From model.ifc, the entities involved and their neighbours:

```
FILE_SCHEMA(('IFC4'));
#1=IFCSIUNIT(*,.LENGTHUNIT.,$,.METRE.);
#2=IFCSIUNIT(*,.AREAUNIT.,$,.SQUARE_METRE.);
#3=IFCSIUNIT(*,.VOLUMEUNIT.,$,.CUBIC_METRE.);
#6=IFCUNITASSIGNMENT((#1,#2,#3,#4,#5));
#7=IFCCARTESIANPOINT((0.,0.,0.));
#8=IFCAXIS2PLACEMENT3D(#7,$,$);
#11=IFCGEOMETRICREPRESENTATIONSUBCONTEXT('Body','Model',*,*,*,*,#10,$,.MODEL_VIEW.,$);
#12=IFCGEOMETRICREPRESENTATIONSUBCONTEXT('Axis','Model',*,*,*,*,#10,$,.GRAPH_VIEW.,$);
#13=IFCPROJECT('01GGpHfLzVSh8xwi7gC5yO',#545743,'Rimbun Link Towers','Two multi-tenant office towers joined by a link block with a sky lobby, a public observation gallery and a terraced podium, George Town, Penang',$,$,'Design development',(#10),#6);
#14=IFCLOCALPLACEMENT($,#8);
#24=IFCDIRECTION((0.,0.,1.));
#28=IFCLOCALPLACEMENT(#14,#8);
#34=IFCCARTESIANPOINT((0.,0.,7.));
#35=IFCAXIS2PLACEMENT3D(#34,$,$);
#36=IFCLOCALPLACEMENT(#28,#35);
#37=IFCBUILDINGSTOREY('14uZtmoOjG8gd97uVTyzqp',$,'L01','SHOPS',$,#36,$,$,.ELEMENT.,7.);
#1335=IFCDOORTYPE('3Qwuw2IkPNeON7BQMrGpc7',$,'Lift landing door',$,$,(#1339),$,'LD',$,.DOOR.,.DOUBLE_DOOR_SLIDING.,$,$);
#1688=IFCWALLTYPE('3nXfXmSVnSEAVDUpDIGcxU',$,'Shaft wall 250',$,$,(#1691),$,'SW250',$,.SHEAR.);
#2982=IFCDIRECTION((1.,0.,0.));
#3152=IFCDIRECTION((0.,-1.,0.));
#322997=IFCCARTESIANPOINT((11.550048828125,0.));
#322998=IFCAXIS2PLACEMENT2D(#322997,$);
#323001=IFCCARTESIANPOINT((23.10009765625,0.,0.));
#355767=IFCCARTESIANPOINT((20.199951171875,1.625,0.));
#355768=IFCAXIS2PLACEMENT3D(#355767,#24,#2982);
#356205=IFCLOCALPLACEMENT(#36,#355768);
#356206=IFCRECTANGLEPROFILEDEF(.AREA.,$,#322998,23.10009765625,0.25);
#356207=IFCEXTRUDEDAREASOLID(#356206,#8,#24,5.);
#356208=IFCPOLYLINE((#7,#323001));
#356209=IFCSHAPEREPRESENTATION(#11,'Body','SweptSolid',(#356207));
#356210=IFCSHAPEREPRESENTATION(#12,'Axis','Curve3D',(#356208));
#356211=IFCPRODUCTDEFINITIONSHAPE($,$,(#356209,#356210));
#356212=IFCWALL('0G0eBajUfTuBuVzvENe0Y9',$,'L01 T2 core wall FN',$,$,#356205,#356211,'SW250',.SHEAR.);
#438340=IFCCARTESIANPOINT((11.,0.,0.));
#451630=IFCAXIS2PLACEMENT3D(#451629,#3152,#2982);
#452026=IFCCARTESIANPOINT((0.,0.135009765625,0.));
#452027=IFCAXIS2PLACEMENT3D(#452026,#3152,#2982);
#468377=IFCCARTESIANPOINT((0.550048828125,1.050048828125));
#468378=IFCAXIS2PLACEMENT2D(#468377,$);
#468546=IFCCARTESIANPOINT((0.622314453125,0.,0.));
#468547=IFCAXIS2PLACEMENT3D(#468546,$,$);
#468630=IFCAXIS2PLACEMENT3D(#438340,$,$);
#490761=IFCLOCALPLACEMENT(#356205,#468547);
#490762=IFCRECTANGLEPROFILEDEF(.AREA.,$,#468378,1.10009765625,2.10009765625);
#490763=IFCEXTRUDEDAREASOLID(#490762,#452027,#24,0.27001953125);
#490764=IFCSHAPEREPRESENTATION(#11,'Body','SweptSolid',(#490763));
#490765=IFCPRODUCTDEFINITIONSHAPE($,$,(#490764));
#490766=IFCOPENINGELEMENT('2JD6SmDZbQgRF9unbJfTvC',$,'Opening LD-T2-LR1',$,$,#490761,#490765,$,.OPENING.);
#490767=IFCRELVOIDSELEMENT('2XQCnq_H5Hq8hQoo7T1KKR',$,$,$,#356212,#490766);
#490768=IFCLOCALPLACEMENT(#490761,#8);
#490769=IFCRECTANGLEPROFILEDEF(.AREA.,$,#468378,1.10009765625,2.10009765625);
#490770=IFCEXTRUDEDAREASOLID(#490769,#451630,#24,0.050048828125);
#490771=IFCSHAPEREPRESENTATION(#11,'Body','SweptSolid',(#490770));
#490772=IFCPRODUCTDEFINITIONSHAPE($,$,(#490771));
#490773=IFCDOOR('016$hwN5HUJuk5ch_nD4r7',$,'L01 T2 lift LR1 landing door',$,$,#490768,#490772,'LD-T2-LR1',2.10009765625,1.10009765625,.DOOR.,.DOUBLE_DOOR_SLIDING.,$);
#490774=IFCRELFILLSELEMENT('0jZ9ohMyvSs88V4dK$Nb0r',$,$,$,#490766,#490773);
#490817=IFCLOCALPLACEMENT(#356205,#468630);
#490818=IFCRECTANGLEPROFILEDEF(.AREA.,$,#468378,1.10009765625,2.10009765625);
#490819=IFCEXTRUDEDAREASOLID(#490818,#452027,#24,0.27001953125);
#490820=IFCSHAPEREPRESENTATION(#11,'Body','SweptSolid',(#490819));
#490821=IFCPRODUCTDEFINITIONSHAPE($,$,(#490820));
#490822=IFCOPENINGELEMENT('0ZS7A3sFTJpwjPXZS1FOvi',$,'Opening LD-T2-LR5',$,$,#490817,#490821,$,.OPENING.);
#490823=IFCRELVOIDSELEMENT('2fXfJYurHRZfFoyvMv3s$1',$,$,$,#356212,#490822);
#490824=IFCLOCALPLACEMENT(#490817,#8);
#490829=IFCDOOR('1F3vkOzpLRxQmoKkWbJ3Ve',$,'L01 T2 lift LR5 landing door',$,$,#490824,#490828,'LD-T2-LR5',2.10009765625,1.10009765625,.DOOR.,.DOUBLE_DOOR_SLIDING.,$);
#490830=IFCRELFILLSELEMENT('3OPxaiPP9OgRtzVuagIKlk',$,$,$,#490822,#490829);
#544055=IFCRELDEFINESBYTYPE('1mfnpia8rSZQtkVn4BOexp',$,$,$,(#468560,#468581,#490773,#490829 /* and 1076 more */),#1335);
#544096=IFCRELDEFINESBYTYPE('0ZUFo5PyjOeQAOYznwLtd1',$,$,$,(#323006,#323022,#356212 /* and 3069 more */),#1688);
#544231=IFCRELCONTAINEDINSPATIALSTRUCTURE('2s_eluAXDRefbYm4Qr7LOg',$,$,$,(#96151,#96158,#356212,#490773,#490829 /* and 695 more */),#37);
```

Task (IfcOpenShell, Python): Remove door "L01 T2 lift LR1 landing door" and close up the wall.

```python
import ifcopenshell
import ifcopenshell.api.feature
import ifcopenshell.api.root
import ifcopenshell.geom
import ifcopenshell.util.shape

model = ifcopenshell.open("model.ifc")
settings = ifcopenshell.geom.settings()


def volume(element):
    """Net volume in cubic metres, openings subtracted."""
    shape = ifcopenshell.geom.create_shape(settings, element)
    return ifcopenshell.util.shape.get_volume(shape.geometry)


door = model.by_id(490773)
opening = door.FillsVoids[0].RelatingOpeningElement
wall = opening.VoidsElements[0].RelatingBuildingElement
before = volume(wall)

ifcopenshell.api.root.remove_product(model, product=door)
ifcopenshell.api.feature.remove_feature(model, feature=opening)

after = volume(wall)

print(f"wall volume {before:.3f} -> {after:.3f} m3")

model.write("model_rev.ifc")
```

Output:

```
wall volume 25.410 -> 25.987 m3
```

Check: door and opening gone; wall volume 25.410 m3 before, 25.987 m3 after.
